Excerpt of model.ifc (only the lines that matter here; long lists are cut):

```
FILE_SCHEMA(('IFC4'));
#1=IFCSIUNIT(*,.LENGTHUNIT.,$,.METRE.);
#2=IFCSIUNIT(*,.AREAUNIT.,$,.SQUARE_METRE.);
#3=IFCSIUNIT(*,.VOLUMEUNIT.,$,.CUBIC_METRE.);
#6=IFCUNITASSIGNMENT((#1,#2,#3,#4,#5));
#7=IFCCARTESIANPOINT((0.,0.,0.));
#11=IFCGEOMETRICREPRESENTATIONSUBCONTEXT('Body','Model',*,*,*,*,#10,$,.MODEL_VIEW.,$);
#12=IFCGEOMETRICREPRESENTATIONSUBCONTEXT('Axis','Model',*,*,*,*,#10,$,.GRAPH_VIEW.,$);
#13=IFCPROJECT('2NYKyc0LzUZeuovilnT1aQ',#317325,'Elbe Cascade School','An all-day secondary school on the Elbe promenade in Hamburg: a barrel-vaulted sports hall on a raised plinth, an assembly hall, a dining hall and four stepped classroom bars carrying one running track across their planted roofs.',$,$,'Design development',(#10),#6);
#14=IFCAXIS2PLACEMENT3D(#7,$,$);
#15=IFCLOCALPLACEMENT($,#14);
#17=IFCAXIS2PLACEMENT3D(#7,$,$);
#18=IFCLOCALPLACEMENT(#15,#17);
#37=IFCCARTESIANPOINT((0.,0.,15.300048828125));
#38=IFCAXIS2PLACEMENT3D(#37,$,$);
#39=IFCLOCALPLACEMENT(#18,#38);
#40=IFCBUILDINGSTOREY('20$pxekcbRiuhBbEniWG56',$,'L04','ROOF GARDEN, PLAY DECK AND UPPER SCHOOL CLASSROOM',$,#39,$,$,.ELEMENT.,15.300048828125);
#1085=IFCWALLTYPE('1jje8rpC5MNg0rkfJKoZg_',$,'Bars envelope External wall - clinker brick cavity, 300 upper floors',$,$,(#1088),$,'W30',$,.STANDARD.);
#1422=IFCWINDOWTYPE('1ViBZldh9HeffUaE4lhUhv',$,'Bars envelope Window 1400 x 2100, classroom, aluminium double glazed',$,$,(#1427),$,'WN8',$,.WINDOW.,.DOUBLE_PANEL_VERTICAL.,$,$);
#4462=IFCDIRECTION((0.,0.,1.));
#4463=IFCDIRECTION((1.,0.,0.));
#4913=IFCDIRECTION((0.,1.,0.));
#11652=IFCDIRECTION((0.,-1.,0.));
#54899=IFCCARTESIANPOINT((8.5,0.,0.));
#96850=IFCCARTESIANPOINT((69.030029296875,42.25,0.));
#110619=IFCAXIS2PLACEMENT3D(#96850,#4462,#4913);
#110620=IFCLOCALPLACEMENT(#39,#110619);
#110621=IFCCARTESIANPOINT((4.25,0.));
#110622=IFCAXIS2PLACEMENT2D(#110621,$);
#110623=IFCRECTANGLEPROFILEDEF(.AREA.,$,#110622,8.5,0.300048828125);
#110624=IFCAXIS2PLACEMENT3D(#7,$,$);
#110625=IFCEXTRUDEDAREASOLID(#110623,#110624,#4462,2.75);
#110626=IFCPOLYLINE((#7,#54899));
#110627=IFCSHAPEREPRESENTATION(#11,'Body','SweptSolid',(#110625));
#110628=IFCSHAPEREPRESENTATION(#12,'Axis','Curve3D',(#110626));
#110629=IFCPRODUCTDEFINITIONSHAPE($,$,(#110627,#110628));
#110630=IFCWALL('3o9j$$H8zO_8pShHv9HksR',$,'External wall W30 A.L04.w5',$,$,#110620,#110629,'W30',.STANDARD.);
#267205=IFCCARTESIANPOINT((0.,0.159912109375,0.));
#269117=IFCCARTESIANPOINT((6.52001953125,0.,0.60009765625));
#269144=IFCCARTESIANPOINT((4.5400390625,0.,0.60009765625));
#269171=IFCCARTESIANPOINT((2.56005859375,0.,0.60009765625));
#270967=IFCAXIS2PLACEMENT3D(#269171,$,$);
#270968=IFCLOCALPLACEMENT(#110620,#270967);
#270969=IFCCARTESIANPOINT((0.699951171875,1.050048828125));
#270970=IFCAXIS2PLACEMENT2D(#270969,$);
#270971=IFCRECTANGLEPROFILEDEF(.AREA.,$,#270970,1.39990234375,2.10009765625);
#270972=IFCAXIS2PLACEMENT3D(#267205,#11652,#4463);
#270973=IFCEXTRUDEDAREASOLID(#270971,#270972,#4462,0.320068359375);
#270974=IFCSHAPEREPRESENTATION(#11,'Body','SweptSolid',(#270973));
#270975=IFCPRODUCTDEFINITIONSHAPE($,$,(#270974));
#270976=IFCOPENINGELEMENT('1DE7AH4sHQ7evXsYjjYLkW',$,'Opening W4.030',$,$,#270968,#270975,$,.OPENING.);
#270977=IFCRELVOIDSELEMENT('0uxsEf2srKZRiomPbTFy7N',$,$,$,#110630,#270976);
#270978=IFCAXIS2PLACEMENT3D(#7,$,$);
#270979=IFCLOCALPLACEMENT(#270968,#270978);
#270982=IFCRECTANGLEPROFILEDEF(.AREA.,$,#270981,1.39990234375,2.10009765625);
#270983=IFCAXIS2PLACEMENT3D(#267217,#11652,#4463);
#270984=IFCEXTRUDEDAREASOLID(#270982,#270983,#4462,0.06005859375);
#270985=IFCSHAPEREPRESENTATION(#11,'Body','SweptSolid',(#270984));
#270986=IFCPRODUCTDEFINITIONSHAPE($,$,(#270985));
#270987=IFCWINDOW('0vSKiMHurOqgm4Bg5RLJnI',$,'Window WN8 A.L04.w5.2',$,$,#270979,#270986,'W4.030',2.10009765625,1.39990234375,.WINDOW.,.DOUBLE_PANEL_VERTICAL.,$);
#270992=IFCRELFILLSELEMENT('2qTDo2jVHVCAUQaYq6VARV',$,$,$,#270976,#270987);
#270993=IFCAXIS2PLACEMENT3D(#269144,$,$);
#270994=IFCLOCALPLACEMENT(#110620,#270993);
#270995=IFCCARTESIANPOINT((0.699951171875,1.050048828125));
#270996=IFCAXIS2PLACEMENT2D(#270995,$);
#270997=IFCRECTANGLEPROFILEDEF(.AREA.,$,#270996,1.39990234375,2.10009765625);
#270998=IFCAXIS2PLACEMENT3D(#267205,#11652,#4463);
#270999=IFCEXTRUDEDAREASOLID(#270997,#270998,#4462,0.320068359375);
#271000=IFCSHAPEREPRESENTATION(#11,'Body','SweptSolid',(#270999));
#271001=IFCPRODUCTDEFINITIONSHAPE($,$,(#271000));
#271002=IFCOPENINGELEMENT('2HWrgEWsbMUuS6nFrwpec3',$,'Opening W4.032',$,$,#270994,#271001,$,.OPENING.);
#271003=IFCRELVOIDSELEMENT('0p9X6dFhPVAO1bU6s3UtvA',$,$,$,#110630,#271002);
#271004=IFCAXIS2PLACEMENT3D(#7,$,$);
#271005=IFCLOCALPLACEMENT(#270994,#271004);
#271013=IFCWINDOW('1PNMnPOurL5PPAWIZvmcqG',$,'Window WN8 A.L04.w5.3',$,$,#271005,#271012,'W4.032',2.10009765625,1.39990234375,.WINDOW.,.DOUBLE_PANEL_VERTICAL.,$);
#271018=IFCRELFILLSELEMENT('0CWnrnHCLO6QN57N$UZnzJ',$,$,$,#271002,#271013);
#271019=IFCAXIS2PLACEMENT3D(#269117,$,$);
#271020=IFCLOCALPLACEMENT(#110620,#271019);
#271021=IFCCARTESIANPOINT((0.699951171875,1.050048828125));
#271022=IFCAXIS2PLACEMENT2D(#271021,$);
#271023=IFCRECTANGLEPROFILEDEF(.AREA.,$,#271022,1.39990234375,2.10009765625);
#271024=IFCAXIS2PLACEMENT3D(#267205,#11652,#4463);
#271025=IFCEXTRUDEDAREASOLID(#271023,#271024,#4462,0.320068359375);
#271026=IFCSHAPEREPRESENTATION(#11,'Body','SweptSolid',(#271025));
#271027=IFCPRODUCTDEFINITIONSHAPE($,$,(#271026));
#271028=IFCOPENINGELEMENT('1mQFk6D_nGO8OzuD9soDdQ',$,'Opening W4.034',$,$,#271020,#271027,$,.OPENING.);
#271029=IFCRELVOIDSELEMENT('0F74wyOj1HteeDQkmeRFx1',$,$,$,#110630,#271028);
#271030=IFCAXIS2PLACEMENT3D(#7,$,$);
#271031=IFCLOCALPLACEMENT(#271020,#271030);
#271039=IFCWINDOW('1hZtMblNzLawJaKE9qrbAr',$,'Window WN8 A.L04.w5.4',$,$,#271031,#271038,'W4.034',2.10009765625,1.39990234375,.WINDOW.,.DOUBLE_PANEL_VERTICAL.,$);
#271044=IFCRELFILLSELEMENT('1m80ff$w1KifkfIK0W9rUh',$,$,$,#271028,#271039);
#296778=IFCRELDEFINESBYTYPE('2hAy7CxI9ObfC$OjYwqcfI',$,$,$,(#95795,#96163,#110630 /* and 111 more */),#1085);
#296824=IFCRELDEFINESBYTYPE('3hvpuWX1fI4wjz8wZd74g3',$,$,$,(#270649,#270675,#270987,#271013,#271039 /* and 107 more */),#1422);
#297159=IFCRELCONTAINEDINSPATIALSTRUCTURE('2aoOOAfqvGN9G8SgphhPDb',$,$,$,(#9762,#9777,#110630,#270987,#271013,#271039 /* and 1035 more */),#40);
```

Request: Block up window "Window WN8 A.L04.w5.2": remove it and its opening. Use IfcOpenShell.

```python
import ifcopenshell
import ifcopenshell.api.feature
import ifcopenshell.api.root
import ifcopenshell.geom
import ifcopenshell.util.shape

model = ifcopenshell.open("model.ifc")
settings = ifcopenshell.geom.settings()


def volume(element):
    """Net volume in cubic metres, openings subtracted."""
    shape = ifcopenshell.geom.create_shape(settings, element)
    return ifcopenshell.util.shape.get_volume(shape.geometry)


window = model.by_guid("0vSKiMHurOqgm4Bg5RLJnI")
opening = window.FillsVoids[0].RelatingOpeningElement
wall = opening.VoidsElements[0].RelatingBuildingElement
before = volume(wall)

ifcopenshell.api.root.remove_product(model, product=window)
ifcopenshell.api.feature.remove_feature(model, feature=opening)

after = volume(wall)

print(f"wall volume {before:.3f} -> {after:.3f} m3")

model.write("model_updated.ifc")
```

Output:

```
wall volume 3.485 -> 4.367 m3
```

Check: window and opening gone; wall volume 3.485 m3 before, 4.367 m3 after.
